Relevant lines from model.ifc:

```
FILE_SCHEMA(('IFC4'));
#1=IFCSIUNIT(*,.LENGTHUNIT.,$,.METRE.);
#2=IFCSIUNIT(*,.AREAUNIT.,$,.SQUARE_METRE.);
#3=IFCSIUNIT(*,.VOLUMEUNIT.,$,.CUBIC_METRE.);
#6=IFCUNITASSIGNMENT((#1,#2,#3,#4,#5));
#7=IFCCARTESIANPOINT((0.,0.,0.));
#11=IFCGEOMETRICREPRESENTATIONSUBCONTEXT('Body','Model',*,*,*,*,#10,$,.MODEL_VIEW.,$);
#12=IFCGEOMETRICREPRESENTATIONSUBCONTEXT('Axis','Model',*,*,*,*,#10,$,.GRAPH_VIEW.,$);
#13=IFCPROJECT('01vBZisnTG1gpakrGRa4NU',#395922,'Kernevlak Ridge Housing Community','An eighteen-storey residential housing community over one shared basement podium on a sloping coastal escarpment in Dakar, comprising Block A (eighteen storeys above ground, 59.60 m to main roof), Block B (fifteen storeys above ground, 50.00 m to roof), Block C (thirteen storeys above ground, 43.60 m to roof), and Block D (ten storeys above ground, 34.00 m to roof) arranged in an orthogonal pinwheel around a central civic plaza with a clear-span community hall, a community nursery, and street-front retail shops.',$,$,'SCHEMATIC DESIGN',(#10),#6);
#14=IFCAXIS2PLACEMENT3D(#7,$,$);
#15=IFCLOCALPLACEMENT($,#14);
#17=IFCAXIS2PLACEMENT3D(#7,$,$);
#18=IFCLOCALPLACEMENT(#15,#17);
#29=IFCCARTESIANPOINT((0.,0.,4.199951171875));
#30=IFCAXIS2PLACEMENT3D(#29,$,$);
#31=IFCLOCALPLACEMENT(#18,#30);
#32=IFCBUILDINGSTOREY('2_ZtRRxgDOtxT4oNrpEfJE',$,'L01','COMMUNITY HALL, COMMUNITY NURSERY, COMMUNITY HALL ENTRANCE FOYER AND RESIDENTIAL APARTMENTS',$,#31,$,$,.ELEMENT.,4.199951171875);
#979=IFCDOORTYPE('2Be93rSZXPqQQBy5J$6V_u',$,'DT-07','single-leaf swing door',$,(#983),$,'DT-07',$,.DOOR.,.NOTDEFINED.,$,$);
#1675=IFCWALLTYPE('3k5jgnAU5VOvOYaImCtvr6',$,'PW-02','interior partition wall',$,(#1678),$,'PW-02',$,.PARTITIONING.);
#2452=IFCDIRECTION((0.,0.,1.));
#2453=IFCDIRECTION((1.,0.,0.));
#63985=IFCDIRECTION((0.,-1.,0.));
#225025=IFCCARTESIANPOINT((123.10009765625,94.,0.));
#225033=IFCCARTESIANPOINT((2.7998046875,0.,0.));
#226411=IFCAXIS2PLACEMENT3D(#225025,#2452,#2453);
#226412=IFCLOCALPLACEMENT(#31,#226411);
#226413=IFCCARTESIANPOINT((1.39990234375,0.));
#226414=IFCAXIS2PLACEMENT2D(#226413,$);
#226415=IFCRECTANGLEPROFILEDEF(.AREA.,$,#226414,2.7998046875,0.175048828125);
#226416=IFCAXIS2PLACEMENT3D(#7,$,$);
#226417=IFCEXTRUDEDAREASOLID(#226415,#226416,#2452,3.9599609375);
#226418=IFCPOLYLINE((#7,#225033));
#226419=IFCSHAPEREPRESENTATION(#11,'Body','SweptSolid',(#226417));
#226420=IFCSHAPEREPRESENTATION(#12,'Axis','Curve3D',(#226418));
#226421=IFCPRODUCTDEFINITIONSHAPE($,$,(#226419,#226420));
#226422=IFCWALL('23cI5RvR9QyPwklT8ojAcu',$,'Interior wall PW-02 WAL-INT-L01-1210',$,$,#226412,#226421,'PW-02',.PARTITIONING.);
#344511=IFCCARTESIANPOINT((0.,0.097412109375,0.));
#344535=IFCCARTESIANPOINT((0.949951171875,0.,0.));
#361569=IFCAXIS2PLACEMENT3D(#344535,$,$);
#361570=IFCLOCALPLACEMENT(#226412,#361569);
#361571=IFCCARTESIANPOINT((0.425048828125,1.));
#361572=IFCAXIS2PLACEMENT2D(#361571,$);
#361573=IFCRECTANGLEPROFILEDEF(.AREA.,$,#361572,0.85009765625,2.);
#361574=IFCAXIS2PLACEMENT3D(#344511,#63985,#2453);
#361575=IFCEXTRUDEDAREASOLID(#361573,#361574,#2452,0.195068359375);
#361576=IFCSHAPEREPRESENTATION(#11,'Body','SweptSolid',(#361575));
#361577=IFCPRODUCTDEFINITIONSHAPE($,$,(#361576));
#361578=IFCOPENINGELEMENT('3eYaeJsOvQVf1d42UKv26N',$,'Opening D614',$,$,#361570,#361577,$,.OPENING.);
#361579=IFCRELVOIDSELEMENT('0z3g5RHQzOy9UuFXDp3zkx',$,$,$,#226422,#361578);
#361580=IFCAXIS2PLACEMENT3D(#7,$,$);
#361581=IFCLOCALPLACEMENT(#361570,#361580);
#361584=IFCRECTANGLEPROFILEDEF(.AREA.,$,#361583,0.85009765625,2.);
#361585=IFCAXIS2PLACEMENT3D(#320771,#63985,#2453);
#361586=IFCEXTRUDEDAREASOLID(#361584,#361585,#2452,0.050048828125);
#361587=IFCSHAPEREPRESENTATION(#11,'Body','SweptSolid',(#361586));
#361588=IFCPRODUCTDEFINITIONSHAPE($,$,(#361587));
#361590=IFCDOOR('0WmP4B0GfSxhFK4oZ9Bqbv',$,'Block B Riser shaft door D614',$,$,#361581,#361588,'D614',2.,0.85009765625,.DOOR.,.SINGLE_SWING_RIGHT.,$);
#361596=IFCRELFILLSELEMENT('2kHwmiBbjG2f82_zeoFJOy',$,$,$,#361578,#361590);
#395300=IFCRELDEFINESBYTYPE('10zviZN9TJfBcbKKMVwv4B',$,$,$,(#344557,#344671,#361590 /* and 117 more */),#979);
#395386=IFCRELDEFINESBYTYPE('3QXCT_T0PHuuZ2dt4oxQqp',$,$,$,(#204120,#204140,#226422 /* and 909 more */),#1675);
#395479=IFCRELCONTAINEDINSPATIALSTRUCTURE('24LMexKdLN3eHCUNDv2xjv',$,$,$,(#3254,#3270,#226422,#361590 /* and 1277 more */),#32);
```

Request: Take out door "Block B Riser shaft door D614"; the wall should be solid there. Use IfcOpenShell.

```python
import ifcopenshell
import ifcopenshell.api.feature
import ifcopenshell.api.root
import ifcopenshell.geom
import ifcopenshell.util.shape

model = ifcopenshell.open("model.ifc")
settings = ifcopenshell.geom.settings()


def volume(element):
    """Net volume in cubic metres, openings subtracted."""
    shape = ifcopenshell.geom.create_shape(settings, element)
    return ifcopenshell.util.shape.get_volume(shape.geometry)


door = model.by_id(361590)
opening = door.FillsVoids[0].RelatingOpeningElement
wall = opening.VoidsElements[0].RelatingBuildingElement
before = volume(wall)

ifcopenshell.api.root.remove_product(model, product=door)
ifcopenshell.api.feature.remove_feature(model, feature=opening)

after = volume(wall)

print(f"wall volume {before:.3f} -> {after:.3f} m3")

model.write("model_v2.ifc")
```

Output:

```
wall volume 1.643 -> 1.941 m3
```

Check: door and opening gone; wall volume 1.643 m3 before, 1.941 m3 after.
